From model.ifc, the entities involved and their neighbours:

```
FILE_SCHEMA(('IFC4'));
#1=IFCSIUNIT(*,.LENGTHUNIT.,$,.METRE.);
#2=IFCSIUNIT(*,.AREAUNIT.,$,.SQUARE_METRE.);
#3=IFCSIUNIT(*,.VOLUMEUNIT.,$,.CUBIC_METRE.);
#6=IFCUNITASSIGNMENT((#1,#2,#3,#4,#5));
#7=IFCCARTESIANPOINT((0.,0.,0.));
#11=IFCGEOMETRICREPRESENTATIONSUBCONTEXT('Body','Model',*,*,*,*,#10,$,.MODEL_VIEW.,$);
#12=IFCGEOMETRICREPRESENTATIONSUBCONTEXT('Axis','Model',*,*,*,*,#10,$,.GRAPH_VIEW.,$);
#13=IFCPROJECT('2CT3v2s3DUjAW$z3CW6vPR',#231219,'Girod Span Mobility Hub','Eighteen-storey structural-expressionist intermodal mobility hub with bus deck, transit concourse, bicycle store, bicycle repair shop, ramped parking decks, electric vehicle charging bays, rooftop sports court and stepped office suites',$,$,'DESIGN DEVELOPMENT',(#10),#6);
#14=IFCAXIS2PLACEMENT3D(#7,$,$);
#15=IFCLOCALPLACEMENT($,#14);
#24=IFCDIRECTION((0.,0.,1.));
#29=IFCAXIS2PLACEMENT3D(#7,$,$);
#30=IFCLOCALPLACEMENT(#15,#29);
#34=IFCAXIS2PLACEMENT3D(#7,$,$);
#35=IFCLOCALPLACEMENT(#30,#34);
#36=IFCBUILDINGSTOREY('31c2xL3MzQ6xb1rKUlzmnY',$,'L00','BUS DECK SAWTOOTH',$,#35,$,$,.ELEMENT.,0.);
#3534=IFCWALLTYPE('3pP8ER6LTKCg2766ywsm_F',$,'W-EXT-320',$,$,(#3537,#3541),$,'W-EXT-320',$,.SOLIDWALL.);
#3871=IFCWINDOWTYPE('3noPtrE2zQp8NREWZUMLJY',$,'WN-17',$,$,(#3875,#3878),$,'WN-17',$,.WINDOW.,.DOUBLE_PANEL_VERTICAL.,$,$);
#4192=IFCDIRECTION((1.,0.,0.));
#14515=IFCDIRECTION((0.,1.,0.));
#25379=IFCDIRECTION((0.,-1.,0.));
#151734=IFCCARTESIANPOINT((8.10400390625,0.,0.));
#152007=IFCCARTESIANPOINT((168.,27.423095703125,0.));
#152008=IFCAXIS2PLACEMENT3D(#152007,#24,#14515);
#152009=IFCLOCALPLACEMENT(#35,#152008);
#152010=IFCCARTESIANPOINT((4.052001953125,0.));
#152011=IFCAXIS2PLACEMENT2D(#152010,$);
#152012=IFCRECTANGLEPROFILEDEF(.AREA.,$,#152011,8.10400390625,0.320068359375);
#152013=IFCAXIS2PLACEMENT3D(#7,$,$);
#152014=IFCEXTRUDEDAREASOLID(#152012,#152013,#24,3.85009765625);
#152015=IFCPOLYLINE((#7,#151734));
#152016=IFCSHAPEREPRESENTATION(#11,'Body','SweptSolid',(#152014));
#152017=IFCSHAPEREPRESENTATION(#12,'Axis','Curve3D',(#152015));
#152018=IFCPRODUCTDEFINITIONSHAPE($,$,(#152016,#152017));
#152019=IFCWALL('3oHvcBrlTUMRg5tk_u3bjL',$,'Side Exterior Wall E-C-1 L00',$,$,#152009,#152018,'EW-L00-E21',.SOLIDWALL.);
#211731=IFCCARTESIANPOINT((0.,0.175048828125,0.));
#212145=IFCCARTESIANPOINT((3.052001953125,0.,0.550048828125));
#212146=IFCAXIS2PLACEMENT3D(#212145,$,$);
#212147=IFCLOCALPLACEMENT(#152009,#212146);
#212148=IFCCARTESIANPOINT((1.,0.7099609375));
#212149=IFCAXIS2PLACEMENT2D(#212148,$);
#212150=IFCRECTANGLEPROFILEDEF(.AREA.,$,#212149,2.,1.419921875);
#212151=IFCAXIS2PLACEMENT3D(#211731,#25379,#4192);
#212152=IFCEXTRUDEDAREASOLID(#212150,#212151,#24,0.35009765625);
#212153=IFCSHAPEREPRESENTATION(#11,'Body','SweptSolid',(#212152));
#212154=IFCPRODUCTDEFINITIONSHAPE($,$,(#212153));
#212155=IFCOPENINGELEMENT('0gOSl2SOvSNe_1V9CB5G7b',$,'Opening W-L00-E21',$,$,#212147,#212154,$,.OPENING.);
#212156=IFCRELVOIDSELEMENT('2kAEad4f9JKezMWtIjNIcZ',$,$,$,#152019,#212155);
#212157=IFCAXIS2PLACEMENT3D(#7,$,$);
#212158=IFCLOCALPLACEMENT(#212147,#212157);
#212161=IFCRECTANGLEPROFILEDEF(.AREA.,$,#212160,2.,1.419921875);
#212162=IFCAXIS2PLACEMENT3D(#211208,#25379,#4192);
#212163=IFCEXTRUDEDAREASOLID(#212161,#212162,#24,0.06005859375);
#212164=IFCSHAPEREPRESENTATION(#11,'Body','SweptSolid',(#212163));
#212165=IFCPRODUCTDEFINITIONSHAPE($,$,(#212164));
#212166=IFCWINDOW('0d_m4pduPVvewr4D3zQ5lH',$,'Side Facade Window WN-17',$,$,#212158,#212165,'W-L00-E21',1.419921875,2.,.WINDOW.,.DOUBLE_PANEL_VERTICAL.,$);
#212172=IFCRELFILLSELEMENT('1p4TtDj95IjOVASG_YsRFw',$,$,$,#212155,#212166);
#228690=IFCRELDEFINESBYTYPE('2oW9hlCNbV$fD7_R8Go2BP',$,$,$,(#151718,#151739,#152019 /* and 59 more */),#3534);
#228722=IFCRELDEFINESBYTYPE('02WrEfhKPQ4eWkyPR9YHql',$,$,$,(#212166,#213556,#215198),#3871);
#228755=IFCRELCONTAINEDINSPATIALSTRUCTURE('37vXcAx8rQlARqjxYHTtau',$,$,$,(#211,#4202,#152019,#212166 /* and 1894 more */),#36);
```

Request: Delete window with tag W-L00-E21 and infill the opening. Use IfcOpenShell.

```python
import ifcopenshell
import ifcopenshell.api.feature
import ifcopenshell.api.root
import ifcopenshell.geom
import ifcopenshell.util.shape

model = ifcopenshell.open("model.ifc")
settings = ifcopenshell.geom.settings()


def volume(element):
    """Net volume in cubic metres, openings subtracted."""
    shape = ifcopenshell.geom.create_shape(settings, element)
    return ifcopenshell.util.shape.get_volume(shape.geometry)


window = model.by_guid("0d_m4pduPVvewr4D3zQ5lH")
opening = window.FillsVoids[0].RelatingOpeningElement
wall = opening.VoidsElements[0].RelatingBuildingElement
before = volume(wall)

ifcopenshell.api.root.remove_product(model, product=window)
ifcopenshell.api.feature.remove_feature(model, feature=opening)

after = volume(wall)

print(f"wall volume {before:.3f} -> {after:.3f} m3")

model.write("model_updated.ifc")
```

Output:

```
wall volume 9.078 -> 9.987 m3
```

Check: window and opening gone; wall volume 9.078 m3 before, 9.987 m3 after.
